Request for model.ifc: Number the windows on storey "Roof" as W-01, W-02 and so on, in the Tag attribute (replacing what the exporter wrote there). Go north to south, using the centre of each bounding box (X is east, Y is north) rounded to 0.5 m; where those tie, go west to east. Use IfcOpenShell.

First a look at what the model holds.

```python
import ifcopenshell
import ifcopenshell.util.element
import ifcopenshell.util.placement

model = ifcopenshell.open("model.ifc")
print(model.schema)
storey = next(s for s in model.by_type("IfcBuildingStorey") if s.Name == "Roof")
windows = [e for e in ifcopenshell.util.element.get_decomposition(storey) if e.is_a("IfcWindow")]
for e in sorted(windows, key=lambda e: e.id()):
    origin = ifcopenshell.util.placement.get_local_placement(e.ObjectPlacement)[:3, 3]
    print(e.id(), e.Tag, e.Name, origin.round(2) + 0.0, sep=" | ")
```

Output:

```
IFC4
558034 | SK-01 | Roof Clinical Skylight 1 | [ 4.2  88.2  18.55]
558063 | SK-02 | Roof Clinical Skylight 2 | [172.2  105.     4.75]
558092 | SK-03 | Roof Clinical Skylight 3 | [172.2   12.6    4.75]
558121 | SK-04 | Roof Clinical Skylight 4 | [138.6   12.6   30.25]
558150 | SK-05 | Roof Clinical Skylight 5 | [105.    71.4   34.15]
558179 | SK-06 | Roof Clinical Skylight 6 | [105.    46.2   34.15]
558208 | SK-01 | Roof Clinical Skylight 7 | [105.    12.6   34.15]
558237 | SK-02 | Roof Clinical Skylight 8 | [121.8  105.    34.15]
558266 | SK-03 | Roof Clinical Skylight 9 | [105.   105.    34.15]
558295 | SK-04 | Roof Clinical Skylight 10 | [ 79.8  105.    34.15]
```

```python
import ifcopenshell
import ifcopenshell.geom
import ifcopenshell.util.element
import ifcopenshell.util.shape

model = ifcopenshell.open("model.ifc")
settings = ifcopenshell.geom.settings()
settings.set("use-world-coords", True)


def centre(element):
    shape = ifcopenshell.geom.create_shape(settings, element)
    return ifcopenshell.util.shape.get_bbox_centroid(shape.geometry)


storey = next(s for s in model.by_type("IfcBuildingStorey") if s.Name == "Roof")
windows = [e for e in ifcopenshell.util.element.get_decomposition(storey) if e.is_a("IfcWindow")]

# Insertion points can sit at a corner or the storey origin, so sort by the geometry (in metres).
centres = {e: centre(e) for e in windows}
windows.sort(key=lambda e: (-round(centres[e][1] / 0.5), centres[e][0]))

for i, e in enumerate(windows, start=1):
    number = f"W-{i:02d}"
    e.Tag = number
    print(e.id(), number)

model.write("model_edited.ifc")
```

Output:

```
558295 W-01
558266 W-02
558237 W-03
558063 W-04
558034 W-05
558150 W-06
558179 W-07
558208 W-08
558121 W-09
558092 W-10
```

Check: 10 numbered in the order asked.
